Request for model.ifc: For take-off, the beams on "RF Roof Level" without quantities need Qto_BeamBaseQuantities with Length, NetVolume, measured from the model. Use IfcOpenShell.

First a look at what the model holds.

```python
import ifcopenshell
import ifcopenshell.util.element
import ifcopenshell.util.unit

model = ifcopenshell.open("model.ifc")
print(model.schema)
for unit_type in ("LENGTHUNIT", "AREAUNIT", "VOLUMEUNIT"):
    print(unit_type, ifcopenshell.util.unit.calculate_unit_scale(model, unit_type))
storey = next(s for s in model.by_type("IfcBuildingStorey") if s.Name == "RF Roof Level")
beams = [e for e in ifcopenshell.util.element.get_decomposition(storey) if e.is_a("IfcBeam")]
for e in sorted(beams, key=lambda e: e.id()):
    print(e.id(), e.is_a(), e.Name, list(ifcopenshell.util.element.get_psets(e, qtos_only=True)), sep=" | ")
```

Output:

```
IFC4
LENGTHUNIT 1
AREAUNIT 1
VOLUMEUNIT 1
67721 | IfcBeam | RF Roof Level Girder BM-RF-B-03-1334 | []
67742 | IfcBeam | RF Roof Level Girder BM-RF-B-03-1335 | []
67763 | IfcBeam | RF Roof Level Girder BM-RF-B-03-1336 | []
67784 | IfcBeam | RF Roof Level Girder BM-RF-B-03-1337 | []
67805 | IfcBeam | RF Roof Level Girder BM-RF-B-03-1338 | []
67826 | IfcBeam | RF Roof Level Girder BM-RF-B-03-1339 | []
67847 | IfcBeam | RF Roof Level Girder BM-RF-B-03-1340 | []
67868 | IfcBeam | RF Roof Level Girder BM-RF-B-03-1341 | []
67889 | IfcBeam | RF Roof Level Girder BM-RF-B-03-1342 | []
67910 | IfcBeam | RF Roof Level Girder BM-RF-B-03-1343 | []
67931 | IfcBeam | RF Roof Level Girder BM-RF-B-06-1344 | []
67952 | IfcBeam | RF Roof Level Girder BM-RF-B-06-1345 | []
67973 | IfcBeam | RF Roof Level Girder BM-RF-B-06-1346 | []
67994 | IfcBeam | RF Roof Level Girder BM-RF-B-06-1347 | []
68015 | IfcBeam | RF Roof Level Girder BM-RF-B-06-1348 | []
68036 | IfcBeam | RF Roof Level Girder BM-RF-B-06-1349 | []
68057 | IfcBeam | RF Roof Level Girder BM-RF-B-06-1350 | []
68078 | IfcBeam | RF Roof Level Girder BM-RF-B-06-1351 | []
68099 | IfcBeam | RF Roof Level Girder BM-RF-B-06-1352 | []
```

```python
import ifcopenshell
import ifcopenshell.api.pset
import ifcopenshell.geom
import ifcopenshell.util.element
import ifcopenshell.util.shape
import ifcopenshell.util.unit

model = ifcopenshell.open("model.ifc")
unit_scale = ifcopenshell.util.unit.calculate_unit_scale(model)
volume_scale = ifcopenshell.util.unit.calculate_unit_scale(model, "VOLUMEUNIT")
settings = ifcopenshell.geom.settings()

storey = next(s for s in model.by_type("IfcBuildingStorey") if s.Name == "RF Roof Level")
beams = [e for e in ifcopenshell.util.element.get_decomposition(storey) if e.is_a("IfcBeam")]

for e in sorted(beams, key=lambda e: e.id()):
    if ifcopenshell.util.element.get_psets(e, qtos_only=True, should_inherit=False):
        continue
    # Geometry comes back in metres, in the element's own axes.
    shape = ifcopenshell.geom.create_shape(settings, e)
    values = {
        "Length": ifcopenshell.util.shape.get_max_xyz(shape.geometry) / unit_scale,
        "NetVolume": ifcopenshell.util.shape.get_volume(shape.geometry) / volume_scale,
    }
    qto = ifcopenshell.api.pset.add_qto(model, product=e, name="Qto_BeamBaseQuantities")
    ifcopenshell.api.pset.edit_qto(model, qto=qto, properties=values)
    print(e.id(), {k: round(v, 3) for k, v in values.items()})

model.write("model_updated.ifc")
```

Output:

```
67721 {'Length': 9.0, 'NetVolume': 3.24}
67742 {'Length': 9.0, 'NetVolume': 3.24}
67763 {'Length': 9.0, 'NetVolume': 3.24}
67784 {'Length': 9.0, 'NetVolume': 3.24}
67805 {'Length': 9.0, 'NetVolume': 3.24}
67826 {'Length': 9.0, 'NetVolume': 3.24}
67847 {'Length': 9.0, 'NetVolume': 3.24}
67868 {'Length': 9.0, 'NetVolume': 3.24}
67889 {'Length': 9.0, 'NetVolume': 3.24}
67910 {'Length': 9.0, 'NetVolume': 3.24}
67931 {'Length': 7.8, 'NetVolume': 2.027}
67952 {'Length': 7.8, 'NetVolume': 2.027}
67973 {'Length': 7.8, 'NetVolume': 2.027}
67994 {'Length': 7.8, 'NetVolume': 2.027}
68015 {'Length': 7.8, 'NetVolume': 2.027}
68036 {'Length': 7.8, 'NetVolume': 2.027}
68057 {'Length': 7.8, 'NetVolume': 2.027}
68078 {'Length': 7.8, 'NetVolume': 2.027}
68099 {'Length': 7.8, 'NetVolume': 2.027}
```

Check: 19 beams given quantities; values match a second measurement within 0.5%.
